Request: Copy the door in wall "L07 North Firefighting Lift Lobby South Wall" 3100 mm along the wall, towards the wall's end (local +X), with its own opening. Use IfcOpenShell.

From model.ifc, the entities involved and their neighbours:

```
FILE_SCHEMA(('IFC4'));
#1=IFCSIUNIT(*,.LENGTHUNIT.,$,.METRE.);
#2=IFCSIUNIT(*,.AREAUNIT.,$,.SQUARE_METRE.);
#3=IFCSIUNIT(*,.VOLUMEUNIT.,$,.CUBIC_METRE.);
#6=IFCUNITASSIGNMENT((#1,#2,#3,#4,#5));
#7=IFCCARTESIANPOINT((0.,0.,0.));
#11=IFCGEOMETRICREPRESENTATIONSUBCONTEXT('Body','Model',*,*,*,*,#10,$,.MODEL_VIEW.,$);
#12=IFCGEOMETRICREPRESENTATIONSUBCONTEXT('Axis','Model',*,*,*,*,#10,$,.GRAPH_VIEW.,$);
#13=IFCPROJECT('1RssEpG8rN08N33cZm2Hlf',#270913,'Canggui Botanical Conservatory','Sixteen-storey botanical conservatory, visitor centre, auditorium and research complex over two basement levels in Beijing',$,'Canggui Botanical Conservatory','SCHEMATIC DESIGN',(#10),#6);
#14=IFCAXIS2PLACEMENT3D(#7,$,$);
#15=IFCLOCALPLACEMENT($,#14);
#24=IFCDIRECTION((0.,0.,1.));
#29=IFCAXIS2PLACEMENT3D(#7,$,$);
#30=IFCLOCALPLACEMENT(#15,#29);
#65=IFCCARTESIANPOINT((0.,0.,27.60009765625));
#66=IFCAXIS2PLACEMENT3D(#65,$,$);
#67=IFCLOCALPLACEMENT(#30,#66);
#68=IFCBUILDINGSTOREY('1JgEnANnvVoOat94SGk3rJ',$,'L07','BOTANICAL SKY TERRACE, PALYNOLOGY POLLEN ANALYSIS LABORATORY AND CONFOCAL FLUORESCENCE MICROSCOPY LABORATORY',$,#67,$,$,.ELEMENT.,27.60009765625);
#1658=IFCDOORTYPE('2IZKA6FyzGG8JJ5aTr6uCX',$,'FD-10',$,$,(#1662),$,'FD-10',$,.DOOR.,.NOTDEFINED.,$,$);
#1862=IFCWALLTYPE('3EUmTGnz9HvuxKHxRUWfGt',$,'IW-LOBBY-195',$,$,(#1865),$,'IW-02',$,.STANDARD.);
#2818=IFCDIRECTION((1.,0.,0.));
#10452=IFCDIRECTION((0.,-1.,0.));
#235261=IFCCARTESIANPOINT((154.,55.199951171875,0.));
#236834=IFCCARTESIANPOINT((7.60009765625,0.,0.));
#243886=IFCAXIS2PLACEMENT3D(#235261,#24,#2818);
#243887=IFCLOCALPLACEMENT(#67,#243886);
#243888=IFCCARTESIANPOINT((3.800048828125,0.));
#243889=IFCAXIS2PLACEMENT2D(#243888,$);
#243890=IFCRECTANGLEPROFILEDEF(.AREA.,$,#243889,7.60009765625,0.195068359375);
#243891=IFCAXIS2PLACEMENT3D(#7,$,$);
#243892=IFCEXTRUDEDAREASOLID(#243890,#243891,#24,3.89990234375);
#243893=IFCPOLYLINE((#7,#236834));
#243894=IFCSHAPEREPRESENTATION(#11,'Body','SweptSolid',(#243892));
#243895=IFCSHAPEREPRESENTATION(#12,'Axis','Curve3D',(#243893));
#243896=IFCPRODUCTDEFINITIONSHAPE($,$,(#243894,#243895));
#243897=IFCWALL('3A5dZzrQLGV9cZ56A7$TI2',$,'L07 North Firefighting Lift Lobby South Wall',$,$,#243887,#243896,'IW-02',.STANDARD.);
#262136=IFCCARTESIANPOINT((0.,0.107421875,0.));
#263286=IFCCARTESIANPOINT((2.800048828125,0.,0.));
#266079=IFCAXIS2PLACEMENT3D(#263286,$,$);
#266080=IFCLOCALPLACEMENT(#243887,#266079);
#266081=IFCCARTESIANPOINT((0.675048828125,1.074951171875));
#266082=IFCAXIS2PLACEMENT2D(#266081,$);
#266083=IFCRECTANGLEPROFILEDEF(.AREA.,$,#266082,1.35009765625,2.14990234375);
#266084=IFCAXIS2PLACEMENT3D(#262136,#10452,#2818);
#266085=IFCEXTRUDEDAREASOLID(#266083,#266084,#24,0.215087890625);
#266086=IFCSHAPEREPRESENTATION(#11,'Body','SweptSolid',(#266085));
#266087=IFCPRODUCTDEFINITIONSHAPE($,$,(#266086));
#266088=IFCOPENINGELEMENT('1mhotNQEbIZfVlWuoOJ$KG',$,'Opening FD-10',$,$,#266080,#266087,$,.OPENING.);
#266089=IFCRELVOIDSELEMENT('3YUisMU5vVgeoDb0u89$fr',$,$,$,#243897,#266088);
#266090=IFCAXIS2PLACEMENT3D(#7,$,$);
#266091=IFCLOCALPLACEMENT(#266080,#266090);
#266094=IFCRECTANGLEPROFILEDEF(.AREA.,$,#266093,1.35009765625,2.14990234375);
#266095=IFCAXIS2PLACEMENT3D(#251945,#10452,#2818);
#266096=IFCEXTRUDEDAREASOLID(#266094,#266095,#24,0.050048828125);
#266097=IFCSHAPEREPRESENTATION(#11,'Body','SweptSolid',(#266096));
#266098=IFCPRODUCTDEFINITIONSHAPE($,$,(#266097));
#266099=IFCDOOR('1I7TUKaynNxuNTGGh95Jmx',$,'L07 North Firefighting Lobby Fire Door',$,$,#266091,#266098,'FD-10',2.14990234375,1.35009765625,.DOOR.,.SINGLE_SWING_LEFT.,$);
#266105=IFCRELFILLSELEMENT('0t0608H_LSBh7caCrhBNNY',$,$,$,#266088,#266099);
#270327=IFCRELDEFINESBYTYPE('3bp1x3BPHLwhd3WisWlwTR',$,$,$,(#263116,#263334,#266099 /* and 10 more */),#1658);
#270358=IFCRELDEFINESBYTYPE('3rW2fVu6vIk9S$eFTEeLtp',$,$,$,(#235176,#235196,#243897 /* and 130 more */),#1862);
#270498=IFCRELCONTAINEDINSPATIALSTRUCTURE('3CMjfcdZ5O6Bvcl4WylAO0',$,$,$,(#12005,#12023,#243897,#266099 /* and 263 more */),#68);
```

```python
import ifcopenshell
import ifcopenshell.api.feature
import ifcopenshell.api.geometry
import ifcopenshell.api.root
import ifcopenshell.geom
import ifcopenshell.util.element
import ifcopenshell.util.placement
import ifcopenshell.util.shape
import ifcopenshell.util.unit

model = ifcopenshell.open("model.ifc")
unit_scale = ifcopenshell.util.unit.calculate_unit_scale(model)
settings = ifcopenshell.geom.settings()


def volume(element):
    """Net volume in cubic metres, openings subtracted."""
    shape = ifcopenshell.geom.create_shape(settings, element)
    return ifcopenshell.util.shape.get_volume(shape.geometry)


door = model.by_guid("1I7TUKaynNxuNTGGh95Jmx")
opening = door.FillsVoids[0].RelatingOpeningElement
wall = opening.VoidsElements[0].RelatingBuildingElement
before = volume(wall)
shift = ifcopenshell.util.placement.get_local_placement(wall.ObjectPlacement)[:3, 0] * 3.1 / unit_scale

# copy_class copies the void relationship, type, container and properties, but no geometry.
new_opening = ifcopenshell.api.root.copy_class(model, product=opening)
new_opening.Representation = ifcopenshell.util.element.copy_deep(
    model, opening.Representation, exclude=["IfcGeometricRepresentationContext", "IfcRepresentationMap"]
)
new_door = ifcopenshell.api.root.copy_class(model, product=door)
new_door.Representation = ifcopenshell.util.element.copy_deep(
    model, door.Representation, exclude=["IfcGeometricRepresentationContext", "IfcRepresentationMap"]
)
new_door.Tag = None
ifcopenshell.api.feature.add_filling(model, opening=new_opening, element=new_door)

for old, new in ((opening, new_opening), (door, new_door)):
    matrix = ifcopenshell.util.placement.get_local_placement(old.ObjectPlacement)
    matrix[:3, 3] += shift
    ifcopenshell.api.geometry.edit_object_placement(model, product=new, matrix=matrix, is_si=False)

after = volume(wall)

print(f"wall volume {before:.3f} -> {after:.3f} m3")

model.write("model_v2.ifc")
```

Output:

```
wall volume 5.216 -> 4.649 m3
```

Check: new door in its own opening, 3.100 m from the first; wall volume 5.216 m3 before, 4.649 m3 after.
